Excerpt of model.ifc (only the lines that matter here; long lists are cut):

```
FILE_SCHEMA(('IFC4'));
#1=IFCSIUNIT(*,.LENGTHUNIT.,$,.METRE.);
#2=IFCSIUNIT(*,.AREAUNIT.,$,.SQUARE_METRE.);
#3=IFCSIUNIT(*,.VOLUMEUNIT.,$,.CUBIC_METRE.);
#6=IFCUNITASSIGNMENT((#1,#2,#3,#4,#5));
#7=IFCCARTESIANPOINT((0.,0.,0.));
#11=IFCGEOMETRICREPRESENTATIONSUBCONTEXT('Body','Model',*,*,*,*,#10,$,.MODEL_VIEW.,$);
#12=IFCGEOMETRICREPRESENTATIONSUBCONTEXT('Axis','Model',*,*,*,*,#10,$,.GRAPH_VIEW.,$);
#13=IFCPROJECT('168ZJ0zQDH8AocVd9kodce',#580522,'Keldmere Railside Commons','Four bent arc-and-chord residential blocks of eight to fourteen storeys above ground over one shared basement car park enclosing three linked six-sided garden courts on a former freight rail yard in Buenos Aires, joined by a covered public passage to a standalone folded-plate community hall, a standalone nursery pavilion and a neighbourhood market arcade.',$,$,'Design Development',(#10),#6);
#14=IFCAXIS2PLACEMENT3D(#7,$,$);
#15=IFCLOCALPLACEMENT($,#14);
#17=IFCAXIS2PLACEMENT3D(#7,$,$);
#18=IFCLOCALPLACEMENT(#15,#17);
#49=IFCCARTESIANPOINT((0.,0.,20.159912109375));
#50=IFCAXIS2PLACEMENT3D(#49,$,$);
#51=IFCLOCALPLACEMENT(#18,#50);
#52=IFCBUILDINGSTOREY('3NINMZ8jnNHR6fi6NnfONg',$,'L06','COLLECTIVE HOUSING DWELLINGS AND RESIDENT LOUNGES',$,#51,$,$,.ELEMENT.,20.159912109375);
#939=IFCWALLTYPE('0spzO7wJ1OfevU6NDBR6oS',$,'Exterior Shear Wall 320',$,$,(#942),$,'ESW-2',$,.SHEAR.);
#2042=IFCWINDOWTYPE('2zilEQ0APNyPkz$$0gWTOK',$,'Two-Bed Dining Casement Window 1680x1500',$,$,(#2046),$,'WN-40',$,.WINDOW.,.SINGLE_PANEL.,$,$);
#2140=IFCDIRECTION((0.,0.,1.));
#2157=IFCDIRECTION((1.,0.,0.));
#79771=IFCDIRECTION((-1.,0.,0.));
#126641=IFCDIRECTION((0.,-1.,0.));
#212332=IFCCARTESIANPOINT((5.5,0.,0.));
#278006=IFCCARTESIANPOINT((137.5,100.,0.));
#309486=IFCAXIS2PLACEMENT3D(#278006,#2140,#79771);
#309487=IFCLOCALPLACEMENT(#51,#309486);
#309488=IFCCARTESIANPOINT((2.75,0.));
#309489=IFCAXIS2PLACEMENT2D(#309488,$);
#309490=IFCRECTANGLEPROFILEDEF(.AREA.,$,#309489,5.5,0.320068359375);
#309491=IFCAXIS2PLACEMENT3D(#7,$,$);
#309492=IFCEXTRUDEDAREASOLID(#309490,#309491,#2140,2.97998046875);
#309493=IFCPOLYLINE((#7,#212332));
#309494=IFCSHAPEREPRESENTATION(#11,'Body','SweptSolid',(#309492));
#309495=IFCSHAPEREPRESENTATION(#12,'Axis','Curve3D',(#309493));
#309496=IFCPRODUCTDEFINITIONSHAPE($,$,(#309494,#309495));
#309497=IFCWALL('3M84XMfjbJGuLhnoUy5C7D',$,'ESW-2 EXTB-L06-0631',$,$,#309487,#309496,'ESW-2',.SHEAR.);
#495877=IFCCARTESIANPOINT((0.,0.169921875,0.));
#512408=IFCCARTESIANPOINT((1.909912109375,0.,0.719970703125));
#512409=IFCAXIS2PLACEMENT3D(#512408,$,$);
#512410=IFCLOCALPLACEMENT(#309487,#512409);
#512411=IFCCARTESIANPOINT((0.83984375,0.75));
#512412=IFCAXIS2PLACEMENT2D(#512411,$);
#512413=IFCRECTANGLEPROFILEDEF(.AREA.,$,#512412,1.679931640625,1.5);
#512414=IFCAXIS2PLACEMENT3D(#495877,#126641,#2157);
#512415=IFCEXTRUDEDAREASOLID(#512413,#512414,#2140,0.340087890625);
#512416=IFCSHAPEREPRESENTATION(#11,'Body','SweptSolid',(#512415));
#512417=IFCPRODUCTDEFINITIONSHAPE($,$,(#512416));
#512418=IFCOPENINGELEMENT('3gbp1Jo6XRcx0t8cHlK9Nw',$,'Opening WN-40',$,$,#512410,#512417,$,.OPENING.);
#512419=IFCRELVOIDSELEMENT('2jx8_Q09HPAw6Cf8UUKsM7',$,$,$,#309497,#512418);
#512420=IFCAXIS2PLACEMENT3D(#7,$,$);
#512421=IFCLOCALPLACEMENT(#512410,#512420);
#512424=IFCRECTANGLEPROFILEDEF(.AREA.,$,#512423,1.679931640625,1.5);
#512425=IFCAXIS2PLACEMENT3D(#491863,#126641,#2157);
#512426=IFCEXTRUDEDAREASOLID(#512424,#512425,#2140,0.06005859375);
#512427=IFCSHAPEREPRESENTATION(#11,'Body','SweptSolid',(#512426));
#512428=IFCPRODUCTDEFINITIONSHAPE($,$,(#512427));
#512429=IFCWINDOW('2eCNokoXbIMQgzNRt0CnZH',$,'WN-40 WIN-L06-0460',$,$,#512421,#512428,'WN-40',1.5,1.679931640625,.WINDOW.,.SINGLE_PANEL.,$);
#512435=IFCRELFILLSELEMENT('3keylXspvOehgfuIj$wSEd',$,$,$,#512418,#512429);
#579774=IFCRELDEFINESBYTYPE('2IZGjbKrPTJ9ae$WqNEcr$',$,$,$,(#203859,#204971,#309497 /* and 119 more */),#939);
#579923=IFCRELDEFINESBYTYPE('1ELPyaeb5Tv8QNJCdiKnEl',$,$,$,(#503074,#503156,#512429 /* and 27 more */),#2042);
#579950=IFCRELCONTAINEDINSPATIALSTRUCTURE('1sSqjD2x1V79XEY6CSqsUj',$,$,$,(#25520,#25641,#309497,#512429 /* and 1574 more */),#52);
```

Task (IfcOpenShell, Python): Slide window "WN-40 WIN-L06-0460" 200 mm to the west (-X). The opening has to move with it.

```python
import ifcopenshell
import ifcopenshell.api.geometry
import ifcopenshell.util.placement

model = ifcopenshell.open("model.ifc")

window = model.by_guid("2eCNokoXbIMQgzNRt0CnZH")
opening = window.FillsVoids[0].RelatingOpeningElement
wall = opening.VoidsElements[0].RelatingBuildingElement

wall_matrix = ifcopenshell.util.placement.get_local_placement(wall.ObjectPlacement)
shift = wall_matrix[:3, 0] * 0.2
before = ifcopenshell.util.placement.get_local_placement(window.ObjectPlacement)[:3, 3].copy()

# The window is placed relative to its opening, so it follows when the opening moves.
matrix = ifcopenshell.util.placement.get_local_placement(opening.ObjectPlacement)
matrix[:3, 3] += shift
ifcopenshell.api.geometry.edit_object_placement(
    model, product=opening, matrix=matrix, is_si=False, should_transform_children=True
)

after = ifcopenshell.util.placement.get_local_placement(window.ObjectPlacement)[:3, 3]
print("window moved by", (after - before).round(3) + 0.0)

model.write("model_edited.ifc")
```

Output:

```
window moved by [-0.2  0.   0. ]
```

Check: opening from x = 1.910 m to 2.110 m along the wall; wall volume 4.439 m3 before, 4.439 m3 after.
